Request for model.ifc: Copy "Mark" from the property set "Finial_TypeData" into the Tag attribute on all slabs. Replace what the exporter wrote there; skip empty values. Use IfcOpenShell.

First a look at what the model holds.

```python
import ifcopenshell
import ifcopenshell.util.element

model = ifcopenshell.open("model.ifc")
print(model.schema)
slabs = model.by_type("IfcSlab")
print(len(slabs), "slabs")
for e in slabs[:8]:
    source = ifcopenshell.util.element.get_pset(e, "Finial_TypeData", "Mark")
    target = e.Tag
    print(e.id(), repr(source), repr(target), sep=" | ")
```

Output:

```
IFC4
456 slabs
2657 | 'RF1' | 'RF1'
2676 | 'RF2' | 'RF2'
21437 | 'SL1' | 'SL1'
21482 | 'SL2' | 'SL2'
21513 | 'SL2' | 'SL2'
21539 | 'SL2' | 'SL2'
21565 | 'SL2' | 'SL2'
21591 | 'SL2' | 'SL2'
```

```python
import ifcopenshell
import ifcopenshell.util.element

model = ifcopenshell.open("model.ifc")

count = 0
for e in model.by_type("IfcSlab"):
    value = ifcopenshell.util.element.get_pset(e, "Finial_TypeData", "Mark")
    current = e.Tag
    if not value or not value.strip() or current == value:
        continue
    e.Tag = value
    count += 1

print(count, "slabs updated")

model.write("model_updated.ifc")
```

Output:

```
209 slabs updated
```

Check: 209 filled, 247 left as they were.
